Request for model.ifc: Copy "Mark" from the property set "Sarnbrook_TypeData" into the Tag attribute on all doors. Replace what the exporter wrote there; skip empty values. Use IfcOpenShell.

First a look at what the model holds.

```python
import ifcopenshell
import ifcopenshell.util.element

model = ifcopenshell.open("model.ifc")
print(model.schema)
doors = model.by_type("IfcDoor")
print(len(doors), "doors")
for e in doors[:8]:
    source = ifcopenshell.util.element.get_pset(e, "Sarnbrook_TypeData", "Mark")
    target = e.Tag
    print(e.id(), repr(source), repr(target), sep=" | ")
```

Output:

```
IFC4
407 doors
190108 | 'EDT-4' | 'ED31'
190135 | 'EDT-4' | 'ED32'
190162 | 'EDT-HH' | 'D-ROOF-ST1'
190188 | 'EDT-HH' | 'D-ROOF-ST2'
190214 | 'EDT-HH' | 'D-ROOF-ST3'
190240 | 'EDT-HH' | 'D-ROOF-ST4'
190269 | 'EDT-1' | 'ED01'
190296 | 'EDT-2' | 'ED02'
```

```python
import ifcopenshell
import ifcopenshell.util.element

model = ifcopenshell.open("model.ifc")

count = 0
for e in model.by_type("IfcDoor"):
    value = ifcopenshell.util.element.get_pset(e, "Sarnbrook_TypeData", "Mark")
    current = e.Tag
    if not value or not value.strip() or current == value:
        continue
    e.Tag = value
    count += 1

print(count, "doors updated")

model.write("model-out.ifc")
```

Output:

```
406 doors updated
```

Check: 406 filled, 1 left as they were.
